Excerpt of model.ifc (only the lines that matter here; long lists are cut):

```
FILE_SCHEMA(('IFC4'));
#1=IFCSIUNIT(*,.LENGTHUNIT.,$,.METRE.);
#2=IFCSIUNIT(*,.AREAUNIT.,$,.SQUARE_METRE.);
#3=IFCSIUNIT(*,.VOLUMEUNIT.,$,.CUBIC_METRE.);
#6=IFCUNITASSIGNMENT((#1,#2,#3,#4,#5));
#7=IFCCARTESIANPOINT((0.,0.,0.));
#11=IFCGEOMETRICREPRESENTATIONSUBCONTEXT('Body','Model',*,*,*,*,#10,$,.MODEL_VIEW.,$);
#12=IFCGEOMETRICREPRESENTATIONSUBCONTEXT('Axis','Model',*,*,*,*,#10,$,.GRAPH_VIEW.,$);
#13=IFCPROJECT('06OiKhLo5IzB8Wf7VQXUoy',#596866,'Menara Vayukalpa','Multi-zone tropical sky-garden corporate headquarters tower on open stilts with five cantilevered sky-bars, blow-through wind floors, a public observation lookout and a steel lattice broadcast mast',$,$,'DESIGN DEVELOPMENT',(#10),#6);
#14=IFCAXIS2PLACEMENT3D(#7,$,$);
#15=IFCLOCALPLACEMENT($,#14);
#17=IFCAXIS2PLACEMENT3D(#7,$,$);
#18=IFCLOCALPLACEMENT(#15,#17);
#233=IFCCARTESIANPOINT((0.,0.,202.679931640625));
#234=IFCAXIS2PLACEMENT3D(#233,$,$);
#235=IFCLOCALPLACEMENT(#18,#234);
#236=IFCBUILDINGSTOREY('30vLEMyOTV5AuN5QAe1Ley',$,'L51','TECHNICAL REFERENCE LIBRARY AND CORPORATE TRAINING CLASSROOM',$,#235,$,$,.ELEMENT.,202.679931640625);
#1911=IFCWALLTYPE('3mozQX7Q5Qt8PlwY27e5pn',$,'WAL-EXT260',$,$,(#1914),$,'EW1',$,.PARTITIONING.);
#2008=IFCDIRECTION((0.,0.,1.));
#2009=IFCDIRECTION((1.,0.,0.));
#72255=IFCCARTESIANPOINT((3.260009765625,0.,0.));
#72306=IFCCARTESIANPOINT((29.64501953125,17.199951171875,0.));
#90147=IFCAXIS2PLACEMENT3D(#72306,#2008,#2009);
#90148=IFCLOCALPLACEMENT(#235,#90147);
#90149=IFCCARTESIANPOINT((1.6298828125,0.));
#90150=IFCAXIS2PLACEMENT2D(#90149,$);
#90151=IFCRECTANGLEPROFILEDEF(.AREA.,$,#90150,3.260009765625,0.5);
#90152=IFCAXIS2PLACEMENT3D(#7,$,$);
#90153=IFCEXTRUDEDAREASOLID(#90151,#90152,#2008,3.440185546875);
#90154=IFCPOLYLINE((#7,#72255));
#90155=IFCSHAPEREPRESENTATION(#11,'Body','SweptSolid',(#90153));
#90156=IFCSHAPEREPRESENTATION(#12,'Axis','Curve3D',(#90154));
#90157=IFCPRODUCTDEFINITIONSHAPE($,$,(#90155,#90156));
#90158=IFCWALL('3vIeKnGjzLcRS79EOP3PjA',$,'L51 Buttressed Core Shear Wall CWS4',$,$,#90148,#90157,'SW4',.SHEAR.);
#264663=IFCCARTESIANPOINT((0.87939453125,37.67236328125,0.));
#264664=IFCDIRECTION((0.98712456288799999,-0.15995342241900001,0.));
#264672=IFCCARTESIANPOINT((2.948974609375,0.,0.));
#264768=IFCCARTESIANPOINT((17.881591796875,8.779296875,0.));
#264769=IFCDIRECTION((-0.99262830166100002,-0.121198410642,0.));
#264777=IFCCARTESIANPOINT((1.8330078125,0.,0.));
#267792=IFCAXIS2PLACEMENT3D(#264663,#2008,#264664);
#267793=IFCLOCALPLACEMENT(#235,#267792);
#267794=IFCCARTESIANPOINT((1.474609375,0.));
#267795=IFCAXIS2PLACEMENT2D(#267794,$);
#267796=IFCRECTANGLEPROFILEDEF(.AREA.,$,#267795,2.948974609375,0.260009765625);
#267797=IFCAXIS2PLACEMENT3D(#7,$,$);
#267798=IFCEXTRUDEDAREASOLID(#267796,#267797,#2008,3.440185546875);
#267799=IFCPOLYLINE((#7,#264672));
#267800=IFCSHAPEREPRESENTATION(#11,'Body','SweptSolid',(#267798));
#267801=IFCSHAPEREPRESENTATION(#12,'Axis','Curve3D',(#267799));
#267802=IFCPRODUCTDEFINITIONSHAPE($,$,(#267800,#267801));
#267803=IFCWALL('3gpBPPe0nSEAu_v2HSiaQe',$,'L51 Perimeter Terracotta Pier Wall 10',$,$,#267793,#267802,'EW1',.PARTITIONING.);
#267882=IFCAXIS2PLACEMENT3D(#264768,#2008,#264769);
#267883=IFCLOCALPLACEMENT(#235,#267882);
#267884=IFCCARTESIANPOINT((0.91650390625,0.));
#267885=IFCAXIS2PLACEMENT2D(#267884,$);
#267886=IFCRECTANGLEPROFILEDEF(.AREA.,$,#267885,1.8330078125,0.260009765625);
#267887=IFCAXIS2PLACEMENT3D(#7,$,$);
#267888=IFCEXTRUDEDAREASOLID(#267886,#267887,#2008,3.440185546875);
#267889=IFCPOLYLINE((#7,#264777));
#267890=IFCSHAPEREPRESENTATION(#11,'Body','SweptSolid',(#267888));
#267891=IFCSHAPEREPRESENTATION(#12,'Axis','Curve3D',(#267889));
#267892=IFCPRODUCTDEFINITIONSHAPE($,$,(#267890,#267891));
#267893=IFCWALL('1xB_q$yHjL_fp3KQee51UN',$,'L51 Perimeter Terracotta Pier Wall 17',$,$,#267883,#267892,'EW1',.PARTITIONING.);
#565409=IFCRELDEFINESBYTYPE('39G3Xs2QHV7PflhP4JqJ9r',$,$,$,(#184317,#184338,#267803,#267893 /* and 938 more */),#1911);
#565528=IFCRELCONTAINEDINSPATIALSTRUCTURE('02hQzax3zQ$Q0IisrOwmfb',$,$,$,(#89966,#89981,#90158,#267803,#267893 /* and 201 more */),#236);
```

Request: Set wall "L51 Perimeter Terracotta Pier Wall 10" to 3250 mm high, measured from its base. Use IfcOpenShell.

```python
import ifcopenshell
import ifcopenshell.geom
import ifcopenshell.util.representation
import ifcopenshell.util.shape
import ifcopenshell.util.unit

model = ifcopenshell.open("model.ifc")
unit_scale = ifcopenshell.util.unit.calculate_unit_scale(model)
settings = ifcopenshell.geom.settings()


def volume(element):
    """Net volume in cubic metres, openings subtracted."""
    shape = ifcopenshell.geom.create_shape(settings, element)
    return ifcopenshell.util.shape.get_volume(shape.geometry)


wall = model.by_guid("3gpBPPe0nSEAu_v2HSiaQe")
before = volume(wall)

body = ifcopenshell.util.representation.get_representation(wall, "Model", "Body")
solid = body.Items[0]
old_height = solid.Depth
solid.Depth = 3.25 / unit_scale
after = volume(wall)

print(f"height {old_height:g} -> {solid.Depth:g}, volume {before:.3f} -> {after:.3f} m3")

model.write("model_edited.ifc")
```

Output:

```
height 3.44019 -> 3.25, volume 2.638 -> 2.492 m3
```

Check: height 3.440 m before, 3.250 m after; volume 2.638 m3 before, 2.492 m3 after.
